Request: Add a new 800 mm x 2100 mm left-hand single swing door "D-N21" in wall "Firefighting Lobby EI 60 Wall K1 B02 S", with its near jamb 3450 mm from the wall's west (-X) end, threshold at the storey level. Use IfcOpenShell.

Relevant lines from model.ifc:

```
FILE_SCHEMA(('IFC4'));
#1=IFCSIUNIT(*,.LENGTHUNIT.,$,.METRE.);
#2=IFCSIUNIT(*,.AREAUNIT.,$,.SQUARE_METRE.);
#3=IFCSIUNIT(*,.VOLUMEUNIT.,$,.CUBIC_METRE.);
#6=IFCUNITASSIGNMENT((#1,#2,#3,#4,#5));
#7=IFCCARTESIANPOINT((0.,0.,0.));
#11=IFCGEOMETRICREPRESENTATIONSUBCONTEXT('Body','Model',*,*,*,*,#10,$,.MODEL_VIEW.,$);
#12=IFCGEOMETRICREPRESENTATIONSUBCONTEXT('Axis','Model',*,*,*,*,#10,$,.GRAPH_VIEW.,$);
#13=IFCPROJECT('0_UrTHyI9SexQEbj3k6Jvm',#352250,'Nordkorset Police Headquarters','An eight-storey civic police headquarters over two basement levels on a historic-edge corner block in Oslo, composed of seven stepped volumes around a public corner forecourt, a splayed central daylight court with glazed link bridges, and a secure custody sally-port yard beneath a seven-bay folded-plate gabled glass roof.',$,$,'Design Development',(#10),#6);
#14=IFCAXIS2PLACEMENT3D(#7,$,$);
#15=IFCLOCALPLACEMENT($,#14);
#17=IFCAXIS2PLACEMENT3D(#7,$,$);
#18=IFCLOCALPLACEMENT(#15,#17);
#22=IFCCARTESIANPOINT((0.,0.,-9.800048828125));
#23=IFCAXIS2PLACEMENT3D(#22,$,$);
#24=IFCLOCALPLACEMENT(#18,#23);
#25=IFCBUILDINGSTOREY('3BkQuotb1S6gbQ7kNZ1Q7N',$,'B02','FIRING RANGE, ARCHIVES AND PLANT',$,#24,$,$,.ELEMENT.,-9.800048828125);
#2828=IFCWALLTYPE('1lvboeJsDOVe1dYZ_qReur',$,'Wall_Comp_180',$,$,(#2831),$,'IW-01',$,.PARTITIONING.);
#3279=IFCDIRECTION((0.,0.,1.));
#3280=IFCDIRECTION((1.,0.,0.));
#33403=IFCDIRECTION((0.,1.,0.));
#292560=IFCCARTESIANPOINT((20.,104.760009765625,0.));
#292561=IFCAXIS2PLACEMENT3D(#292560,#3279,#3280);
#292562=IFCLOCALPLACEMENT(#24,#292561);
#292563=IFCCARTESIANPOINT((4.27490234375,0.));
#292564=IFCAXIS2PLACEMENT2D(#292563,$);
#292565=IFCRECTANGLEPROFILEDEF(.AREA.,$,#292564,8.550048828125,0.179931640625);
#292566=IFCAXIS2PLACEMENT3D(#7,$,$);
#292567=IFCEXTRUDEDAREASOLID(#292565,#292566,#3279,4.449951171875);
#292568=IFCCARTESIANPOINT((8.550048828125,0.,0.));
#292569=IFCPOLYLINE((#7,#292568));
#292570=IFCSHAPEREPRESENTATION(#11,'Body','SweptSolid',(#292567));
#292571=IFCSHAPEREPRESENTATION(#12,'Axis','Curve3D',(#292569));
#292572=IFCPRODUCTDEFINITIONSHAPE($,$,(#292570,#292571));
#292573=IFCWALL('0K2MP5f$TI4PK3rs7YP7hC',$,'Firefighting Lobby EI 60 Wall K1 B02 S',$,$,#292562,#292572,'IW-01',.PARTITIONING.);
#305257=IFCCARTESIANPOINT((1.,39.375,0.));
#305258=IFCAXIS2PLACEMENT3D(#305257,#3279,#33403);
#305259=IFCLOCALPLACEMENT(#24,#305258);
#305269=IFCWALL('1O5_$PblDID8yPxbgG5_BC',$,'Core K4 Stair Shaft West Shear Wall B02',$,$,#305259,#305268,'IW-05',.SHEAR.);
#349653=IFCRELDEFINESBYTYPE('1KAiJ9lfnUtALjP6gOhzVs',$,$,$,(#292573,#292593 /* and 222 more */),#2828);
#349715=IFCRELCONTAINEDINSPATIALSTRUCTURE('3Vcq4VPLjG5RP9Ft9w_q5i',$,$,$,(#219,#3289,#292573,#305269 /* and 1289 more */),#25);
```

```python
import numpy as np
import ifcopenshell
import ifcopenshell.api.feature
import ifcopenshell.api.geometry
import ifcopenshell.api.root
import ifcopenshell.api.spatial
import ifcopenshell.geom
import ifcopenshell.util.element
import ifcopenshell.util.placement
import ifcopenshell.util.representation
import ifcopenshell.util.shape
import ifcopenshell.util.unit

model = ifcopenshell.open("model.ifc")
unit_scale = ifcopenshell.util.unit.calculate_unit_scale(model)
settings = ifcopenshell.geom.settings()


def volume(element):
    """Net volume in cubic metres, openings subtracted."""
    shape = ifcopenshell.geom.create_shape(settings, element)
    return ifcopenshell.util.shape.get_volume(shape.geometry)


wall = model.by_guid("0K2MP5f$TI4PK3rs7YP7hC")
storey = ifcopenshell.util.element.get_container(wall, ifc_class="IfcBuildingStorey")
context = ifcopenshell.util.representation.get_context(model, "Model", "Body", "MODEL_VIEW")
before = volume(wall)

width, height, from_end, sill = 0.8, 2.1, 3.45, 0.0  # metres

# The wall runs along its own X axis, and the end named is its -X end.
wall_shape = ifcopenshell.geom.create_shape(settings, wall)
x, y, z = ifcopenshell.util.shape.get_vertices(wall_shape.geometry).T
start = x.min() + from_end
face, thickness = float(y.min()), float(y.max() - y.min())
wall_matrix = ifcopenshell.util.placement.get_local_placement(wall.ObjectPlacement)
level = ifcopenshell.util.placement.get_local_placement(storey.ObjectPlacement)[2, 3]


def in_wall(x, y):
    """Placement at x, y metres in the wall's axes, at sill height."""
    matrix = wall_matrix.copy()
    matrix[:, 3] = wall_matrix @ np.array([x / unit_scale, y / unit_scale, 0.0, 1.0])
    matrix[2, 3] = level + sill / unit_scale
    return matrix


# Opening: a box that overshoots both wall faces by 50 mm.
opening = ifcopenshell.api.root.create_entity(model, ifc_class="IfcOpeningElement", predefined_type="OPENING")
box = ifcopenshell.api.geometry.add_wall_representation(
    model, context=context, length=width, height=height, thickness=thickness + 0.1
)
ifcopenshell.api.geometry.assign_representation(model, product=opening, representation=box)
ifcopenshell.api.geometry.edit_object_placement(model, product=opening, matrix=in_wall(start, face - 0.05), is_si=False)
ifcopenshell.api.feature.add_feature(model, feature=opening, element=wall)

door = ifcopenshell.api.root.create_entity(model, ifc_class="IfcDoor", name="D-N21", predefined_type="DOOR")
door.OverallWidth, door.OverallHeight = width / unit_scale, height / unit_scale
door.OperationType = "SINGLE_SWING_LEFT"
body = ifcopenshell.api.geometry.add_door_representation(
    model,
    context=context,
    overall_width=door.OverallWidth,
    overall_height=door.OverallHeight,
    operation_type="SINGLE_SWING_LEFT",
    lining_properties={"LiningDepth": thickness / unit_scale, "ThresholdDepth": thickness / unit_scale},
)
ifcopenshell.api.geometry.assign_representation(model, product=door, representation=body)
ifcopenshell.api.spatial.assign_container(model, products=[door], relating_structure=storey)
ifcopenshell.api.feature.add_filling(model, opening=opening, element=door)

# The lining spans the wall, so the door starts at the wall face.
ifcopenshell.api.geometry.edit_object_placement(model, product=door, matrix=in_wall(start, face), is_si=False)

after = volume(wall)

print(f"wall volume {before:.3f} -> {after:.3f} m3")

model.write("model_v2.ifc")
```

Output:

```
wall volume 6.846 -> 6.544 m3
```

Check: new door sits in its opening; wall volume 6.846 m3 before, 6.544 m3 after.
